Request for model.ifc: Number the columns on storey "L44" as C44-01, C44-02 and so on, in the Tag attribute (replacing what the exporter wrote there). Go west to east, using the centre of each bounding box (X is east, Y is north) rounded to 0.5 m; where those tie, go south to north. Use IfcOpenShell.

First a look at what the model holds.

```python
import ifcopenshell
import ifcopenshell.util.element
import ifcopenshell.util.placement

model = ifcopenshell.open("model.ifc")
print(model.schema)
storey = next(s for s in model.by_type("IfcBuildingStorey") if s.Name == "L44")
columns = [e for e in ifcopenshell.util.element.get_decomposition(storey) if e.is_a("IfcColumn")]
for e in sorted(columns, key=lambda e: e.id()):
    origin = ifcopenshell.util.placement.get_local_placement(e.ObjectPlacement)[:3, 3]
    print(e.id(), e.Tag, e.Name, origin.round(2) + 0.0, sep=" | ")
```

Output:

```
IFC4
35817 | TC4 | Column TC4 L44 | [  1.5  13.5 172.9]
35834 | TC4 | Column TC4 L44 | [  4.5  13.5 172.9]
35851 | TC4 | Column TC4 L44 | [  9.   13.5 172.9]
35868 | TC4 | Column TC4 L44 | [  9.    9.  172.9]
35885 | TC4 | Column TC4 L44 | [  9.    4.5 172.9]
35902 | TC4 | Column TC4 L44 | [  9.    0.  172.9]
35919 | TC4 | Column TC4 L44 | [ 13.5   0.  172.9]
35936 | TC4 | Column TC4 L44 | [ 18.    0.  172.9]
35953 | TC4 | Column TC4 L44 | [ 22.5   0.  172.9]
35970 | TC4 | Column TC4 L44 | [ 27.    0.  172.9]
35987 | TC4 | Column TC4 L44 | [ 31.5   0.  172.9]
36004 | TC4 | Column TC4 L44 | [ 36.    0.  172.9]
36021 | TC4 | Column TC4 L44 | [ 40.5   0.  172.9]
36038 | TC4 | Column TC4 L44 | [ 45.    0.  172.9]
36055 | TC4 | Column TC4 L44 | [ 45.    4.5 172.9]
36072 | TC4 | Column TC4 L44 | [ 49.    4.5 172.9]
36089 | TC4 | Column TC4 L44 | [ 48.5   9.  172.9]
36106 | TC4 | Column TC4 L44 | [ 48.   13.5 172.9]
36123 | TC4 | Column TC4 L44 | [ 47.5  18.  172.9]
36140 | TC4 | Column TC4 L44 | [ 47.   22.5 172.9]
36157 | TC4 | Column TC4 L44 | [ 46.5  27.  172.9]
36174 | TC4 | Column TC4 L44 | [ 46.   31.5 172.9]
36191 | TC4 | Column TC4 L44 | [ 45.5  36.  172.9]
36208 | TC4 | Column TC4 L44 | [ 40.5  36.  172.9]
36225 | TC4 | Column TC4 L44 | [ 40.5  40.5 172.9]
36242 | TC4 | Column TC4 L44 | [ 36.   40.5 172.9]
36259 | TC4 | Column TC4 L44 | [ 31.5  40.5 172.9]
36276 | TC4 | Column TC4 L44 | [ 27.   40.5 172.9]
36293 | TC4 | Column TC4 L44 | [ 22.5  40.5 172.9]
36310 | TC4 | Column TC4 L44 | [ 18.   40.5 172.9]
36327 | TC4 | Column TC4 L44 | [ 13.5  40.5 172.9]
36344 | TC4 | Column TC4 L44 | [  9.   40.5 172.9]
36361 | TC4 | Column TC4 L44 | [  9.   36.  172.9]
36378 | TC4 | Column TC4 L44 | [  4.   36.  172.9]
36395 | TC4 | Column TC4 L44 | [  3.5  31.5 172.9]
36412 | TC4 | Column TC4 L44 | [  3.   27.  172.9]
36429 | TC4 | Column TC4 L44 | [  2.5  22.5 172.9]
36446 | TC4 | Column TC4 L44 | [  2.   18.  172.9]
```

```python
import ifcopenshell
import ifcopenshell.geom
import ifcopenshell.util.element
import ifcopenshell.util.shape

model = ifcopenshell.open("model.ifc")
settings = ifcopenshell.geom.settings()
settings.set("use-world-coords", True)


def centre(element):
    shape = ifcopenshell.geom.create_shape(settings, element)
    return ifcopenshell.util.shape.get_bbox_centroid(shape.geometry)


storey = next(s for s in model.by_type("IfcBuildingStorey") if s.Name == "L44")
columns = [e for e in ifcopenshell.util.element.get_decomposition(storey) if e.is_a("IfcColumn")]

# Insertion points can sit at a corner or the storey origin, so sort by the geometry (in metres).
centres = {e: centre(e) for e in columns}
columns.sort(key=lambda e: (round(centres[e][0] / 0.5), centres[e][1]))

for i, e in enumerate(columns, start=1):
    number = f"C44-{i:02d}"
    e.Tag = number
    print(e.id(), number)

model.write("model_rev.ifc")
```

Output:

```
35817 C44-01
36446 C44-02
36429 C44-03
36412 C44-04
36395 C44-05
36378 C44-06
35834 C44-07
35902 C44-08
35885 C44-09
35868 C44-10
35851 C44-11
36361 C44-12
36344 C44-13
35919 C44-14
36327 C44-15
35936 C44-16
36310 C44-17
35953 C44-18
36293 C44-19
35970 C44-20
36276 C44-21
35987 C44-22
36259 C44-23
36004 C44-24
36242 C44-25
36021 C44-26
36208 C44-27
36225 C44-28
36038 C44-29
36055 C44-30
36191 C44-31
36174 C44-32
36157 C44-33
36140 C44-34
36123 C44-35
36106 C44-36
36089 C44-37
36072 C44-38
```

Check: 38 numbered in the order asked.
